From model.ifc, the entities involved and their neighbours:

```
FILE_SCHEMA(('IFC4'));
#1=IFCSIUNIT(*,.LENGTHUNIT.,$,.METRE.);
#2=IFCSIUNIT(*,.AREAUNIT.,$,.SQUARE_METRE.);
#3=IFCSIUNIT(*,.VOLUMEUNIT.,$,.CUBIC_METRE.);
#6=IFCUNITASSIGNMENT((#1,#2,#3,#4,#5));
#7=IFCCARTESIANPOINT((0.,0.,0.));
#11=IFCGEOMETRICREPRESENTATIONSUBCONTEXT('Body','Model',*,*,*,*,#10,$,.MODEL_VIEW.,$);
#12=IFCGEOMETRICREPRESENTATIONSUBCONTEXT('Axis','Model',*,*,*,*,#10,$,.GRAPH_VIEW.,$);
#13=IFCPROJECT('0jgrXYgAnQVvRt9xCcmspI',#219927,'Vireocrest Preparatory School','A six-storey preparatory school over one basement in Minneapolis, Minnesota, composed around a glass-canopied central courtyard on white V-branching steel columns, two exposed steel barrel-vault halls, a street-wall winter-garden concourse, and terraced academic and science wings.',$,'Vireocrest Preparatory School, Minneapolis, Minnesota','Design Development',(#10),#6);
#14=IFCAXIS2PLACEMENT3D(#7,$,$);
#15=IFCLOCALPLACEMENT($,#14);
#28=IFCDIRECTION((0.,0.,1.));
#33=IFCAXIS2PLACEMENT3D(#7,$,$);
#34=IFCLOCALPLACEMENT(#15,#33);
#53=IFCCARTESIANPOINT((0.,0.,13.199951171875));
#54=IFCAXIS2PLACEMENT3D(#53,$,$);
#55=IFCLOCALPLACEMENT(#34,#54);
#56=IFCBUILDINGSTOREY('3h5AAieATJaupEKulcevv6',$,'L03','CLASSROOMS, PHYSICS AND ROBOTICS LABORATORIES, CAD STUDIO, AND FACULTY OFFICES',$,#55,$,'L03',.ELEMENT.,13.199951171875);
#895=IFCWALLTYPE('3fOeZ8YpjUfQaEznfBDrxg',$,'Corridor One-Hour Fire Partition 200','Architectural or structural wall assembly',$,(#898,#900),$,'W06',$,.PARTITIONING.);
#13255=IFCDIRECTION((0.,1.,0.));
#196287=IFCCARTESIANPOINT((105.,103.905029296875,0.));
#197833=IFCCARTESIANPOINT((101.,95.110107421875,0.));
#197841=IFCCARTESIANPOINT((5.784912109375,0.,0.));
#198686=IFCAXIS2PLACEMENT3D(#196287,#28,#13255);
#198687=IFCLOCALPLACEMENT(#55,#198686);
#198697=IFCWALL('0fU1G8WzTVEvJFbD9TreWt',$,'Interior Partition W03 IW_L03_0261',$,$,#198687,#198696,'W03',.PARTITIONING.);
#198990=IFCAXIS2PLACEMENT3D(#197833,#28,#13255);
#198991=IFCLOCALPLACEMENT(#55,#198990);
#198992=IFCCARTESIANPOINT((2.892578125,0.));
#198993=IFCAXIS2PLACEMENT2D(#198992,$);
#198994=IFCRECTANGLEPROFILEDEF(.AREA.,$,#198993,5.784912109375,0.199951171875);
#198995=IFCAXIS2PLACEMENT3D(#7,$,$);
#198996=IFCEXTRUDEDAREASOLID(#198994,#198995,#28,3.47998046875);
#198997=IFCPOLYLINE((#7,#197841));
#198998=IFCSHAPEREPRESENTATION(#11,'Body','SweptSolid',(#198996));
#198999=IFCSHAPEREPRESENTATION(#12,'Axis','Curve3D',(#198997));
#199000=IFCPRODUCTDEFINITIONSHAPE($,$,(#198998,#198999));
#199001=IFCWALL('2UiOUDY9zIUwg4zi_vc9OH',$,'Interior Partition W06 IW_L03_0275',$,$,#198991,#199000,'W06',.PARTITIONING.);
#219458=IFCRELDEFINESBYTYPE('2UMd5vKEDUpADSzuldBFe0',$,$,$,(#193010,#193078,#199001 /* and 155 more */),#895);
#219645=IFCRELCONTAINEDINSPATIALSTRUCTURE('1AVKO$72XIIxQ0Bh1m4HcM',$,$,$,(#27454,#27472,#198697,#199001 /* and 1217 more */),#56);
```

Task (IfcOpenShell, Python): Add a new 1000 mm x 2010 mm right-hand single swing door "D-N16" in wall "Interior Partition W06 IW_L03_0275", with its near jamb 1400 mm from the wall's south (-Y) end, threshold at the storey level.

```python
import numpy as np
import ifcopenshell
import ifcopenshell.api.feature
import ifcopenshell.api.geometry
import ifcopenshell.api.root
import ifcopenshell.api.spatial
import ifcopenshell.geom
import ifcopenshell.util.element
import ifcopenshell.util.placement
import ifcopenshell.util.representation
import ifcopenshell.util.shape
import ifcopenshell.util.unit

model = ifcopenshell.open("model.ifc")
unit_scale = ifcopenshell.util.unit.calculate_unit_scale(model)
settings = ifcopenshell.geom.settings()


def volume(element):
    """Net volume in cubic metres, openings subtracted."""
    shape = ifcopenshell.geom.create_shape(settings, element)
    return ifcopenshell.util.shape.get_volume(shape.geometry)


wall = model.by_id(199001)
storey = ifcopenshell.util.element.get_container(wall, ifc_class="IfcBuildingStorey")
context = ifcopenshell.util.representation.get_context(model, "Model", "Body", "MODEL_VIEW")
before = volume(wall)

width, height, from_end, sill = 1, 2.01, 1.4, 0.0  # metres

# The wall runs along its own X axis, and the end named is its -X end.
wall_shape = ifcopenshell.geom.create_shape(settings, wall)
x, y, z = ifcopenshell.util.shape.get_vertices(wall_shape.geometry).T
start = x.min() + from_end
face, thickness = float(y.min()), float(y.max() - y.min())
wall_matrix = ifcopenshell.util.placement.get_local_placement(wall.ObjectPlacement)
level = ifcopenshell.util.placement.get_local_placement(storey.ObjectPlacement)[2, 3]


def in_wall(x, y):
    """Placement at x, y metres in the wall's axes, at sill height."""
    matrix = wall_matrix.copy()
    matrix[:, 3] = wall_matrix @ np.array([x / unit_scale, y / unit_scale, 0.0, 1.0])
    matrix[2, 3] = level + sill / unit_scale
    return matrix


# Opening: a box that overshoots both wall faces by 50 mm.
opening = ifcopenshell.api.root.create_entity(model, ifc_class="IfcOpeningElement", predefined_type="OPENING")
box = ifcopenshell.api.geometry.add_wall_representation(
    model, context=context, length=width, height=height, thickness=thickness + 0.1
)
ifcopenshell.api.geometry.assign_representation(model, product=opening, representation=box)
ifcopenshell.api.geometry.edit_object_placement(model, product=opening, matrix=in_wall(start, face - 0.05), is_si=False)
ifcopenshell.api.feature.add_feature(model, feature=opening, element=wall)

door = ifcopenshell.api.root.create_entity(model, ifc_class="IfcDoor", name="D-N16", predefined_type="DOOR")
door.OverallWidth, door.OverallHeight = width / unit_scale, height / unit_scale
door.OperationType = "SINGLE_SWING_RIGHT"
body = ifcopenshell.api.geometry.add_door_representation(
    model,
    context=context,
    overall_width=door.OverallWidth,
    overall_height=door.OverallHeight,
    operation_type="SINGLE_SWING_RIGHT",
    lining_properties={"LiningDepth": thickness / unit_scale, "ThresholdDepth": thickness / unit_scale},
)
ifcopenshell.api.geometry.assign_representation(model, product=door, representation=body)
ifcopenshell.api.spatial.assign_container(model, products=[door], relating_structure=storey)
ifcopenshell.api.feature.add_filling(model, opening=opening, element=door)

# The lining spans the wall, so the door starts at the wall face.
ifcopenshell.api.geometry.edit_object_placement(model, product=door, matrix=in_wall(start, face), is_si=False)

after = volume(wall)

print(f"wall volume {before:.3f} -> {after:.3f} m3")

model.write("model-out.ifc")
```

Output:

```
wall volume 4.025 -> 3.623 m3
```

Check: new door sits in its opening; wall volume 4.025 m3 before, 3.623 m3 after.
